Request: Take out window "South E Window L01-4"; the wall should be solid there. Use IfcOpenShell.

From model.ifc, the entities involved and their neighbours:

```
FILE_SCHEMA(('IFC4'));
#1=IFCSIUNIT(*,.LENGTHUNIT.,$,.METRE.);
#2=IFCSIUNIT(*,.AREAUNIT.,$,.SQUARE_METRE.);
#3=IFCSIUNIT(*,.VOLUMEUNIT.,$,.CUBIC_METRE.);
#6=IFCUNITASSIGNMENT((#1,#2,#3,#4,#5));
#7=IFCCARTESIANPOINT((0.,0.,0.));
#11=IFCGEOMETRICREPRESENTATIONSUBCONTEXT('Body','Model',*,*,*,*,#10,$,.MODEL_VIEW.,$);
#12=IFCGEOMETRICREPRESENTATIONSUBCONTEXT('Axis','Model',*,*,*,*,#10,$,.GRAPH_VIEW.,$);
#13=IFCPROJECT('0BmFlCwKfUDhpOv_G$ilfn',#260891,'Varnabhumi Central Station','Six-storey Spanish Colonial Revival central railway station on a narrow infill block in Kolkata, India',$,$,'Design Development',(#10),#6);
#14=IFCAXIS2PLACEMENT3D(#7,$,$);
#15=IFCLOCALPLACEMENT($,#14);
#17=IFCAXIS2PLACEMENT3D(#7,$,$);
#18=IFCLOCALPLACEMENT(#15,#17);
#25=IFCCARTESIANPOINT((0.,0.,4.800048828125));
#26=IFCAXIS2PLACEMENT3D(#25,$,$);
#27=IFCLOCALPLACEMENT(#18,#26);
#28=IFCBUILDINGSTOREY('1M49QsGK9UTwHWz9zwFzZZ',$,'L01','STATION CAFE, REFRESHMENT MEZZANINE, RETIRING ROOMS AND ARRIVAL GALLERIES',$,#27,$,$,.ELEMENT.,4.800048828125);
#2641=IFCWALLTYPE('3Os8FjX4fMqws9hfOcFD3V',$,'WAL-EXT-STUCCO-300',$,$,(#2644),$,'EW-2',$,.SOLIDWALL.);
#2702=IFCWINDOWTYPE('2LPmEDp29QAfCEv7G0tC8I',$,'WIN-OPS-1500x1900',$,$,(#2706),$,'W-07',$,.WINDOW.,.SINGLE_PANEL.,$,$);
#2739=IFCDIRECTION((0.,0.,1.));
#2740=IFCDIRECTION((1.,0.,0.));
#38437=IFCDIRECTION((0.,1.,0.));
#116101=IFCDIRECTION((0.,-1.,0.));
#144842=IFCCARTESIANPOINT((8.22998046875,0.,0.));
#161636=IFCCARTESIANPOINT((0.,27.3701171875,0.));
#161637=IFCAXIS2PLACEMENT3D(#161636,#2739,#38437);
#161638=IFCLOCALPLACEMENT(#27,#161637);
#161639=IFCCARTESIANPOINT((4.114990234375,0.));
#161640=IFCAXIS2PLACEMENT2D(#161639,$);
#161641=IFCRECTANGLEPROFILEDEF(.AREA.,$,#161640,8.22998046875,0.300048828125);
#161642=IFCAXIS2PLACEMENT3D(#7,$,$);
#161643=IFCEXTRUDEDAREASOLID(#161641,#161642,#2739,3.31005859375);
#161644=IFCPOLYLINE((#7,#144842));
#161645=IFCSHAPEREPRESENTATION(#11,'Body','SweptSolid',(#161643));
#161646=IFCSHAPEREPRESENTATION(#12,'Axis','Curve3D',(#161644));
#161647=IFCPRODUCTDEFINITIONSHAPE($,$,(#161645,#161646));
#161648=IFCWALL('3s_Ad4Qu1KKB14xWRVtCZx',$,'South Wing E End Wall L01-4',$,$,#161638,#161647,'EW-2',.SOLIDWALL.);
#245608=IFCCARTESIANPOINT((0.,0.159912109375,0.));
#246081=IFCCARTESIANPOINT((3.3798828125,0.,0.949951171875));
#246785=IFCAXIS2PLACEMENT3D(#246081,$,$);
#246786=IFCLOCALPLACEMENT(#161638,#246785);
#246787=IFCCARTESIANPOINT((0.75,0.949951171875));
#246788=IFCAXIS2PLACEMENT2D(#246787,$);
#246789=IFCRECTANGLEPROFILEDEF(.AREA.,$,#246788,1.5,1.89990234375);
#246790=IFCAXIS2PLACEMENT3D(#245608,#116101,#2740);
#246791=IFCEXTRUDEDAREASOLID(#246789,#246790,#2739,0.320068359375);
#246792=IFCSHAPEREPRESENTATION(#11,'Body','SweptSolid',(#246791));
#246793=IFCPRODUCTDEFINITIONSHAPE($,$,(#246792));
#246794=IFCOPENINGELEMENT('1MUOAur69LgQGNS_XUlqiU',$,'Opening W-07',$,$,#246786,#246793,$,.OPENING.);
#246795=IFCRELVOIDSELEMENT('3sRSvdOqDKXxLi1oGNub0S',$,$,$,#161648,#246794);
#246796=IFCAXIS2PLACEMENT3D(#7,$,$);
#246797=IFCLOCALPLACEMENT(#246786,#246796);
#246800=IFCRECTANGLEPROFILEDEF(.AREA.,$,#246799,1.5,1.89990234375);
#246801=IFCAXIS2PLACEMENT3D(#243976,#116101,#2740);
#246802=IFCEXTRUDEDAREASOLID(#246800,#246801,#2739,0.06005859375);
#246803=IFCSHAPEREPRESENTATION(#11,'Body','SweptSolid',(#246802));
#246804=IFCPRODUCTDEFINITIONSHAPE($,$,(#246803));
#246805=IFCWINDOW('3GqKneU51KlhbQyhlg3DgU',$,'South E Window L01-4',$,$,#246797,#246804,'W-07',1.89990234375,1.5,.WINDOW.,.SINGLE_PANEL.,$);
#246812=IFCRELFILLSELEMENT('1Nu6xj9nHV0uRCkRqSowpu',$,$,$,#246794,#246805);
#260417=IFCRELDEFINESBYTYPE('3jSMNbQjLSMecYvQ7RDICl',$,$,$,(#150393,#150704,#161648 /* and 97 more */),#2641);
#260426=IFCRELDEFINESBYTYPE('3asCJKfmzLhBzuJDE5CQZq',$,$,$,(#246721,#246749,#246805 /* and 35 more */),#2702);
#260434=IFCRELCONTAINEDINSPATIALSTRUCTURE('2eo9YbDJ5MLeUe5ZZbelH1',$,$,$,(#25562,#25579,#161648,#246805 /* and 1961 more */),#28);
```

```python
import ifcopenshell
import ifcopenshell.api.feature
import ifcopenshell.api.root
import ifcopenshell.geom
import ifcopenshell.util.shape

model = ifcopenshell.open("model.ifc")
settings = ifcopenshell.geom.settings()


def volume(element):
    """Net volume in cubic metres, openings subtracted."""
    shape = ifcopenshell.geom.create_shape(settings, element)
    return ifcopenshell.util.shape.get_volume(shape.geometry)


window = model.by_guid("3GqKneU51KlhbQyhlg3DgU")
opening = window.FillsVoids[0].RelatingOpeningElement
wall = opening.VoidsElements[0].RelatingBuildingElement
before = volume(wall)

ifcopenshell.api.root.remove_product(model, product=window)
ifcopenshell.api.feature.remove_feature(model, feature=opening)

after = volume(wall)

print(f"wall volume {before:.3f} -> {after:.3f} m3")

model.write("model_v2.ifc")
```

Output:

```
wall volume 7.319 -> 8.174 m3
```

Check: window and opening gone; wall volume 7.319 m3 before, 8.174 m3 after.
